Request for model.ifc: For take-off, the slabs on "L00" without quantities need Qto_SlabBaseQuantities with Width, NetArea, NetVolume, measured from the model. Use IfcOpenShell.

First a look at what the model holds.

```python
import ifcopenshell
import ifcopenshell.util.element
import ifcopenshell.util.unit

model = ifcopenshell.open("model.ifc")
print(model.schema)
for unit_type in ("LENGTHUNIT", "AREAUNIT", "VOLUMEUNIT"):
    print(unit_type, ifcopenshell.util.unit.calculate_unit_scale(model, unit_type))
storey = next(s for s in model.by_type("IfcBuildingStorey") if s.Name == "L00")
slabs = [e for e in ifcopenshell.util.element.get_decomposition(storey) if e.is_a("IfcSlab")]
for e in sorted(slabs, key=lambda e: e.id()):
    print(e.id(), e.is_a(), e.Name, list(ifcopenshell.util.element.get_psets(e, qtos_only=True)), sep=" | ")
```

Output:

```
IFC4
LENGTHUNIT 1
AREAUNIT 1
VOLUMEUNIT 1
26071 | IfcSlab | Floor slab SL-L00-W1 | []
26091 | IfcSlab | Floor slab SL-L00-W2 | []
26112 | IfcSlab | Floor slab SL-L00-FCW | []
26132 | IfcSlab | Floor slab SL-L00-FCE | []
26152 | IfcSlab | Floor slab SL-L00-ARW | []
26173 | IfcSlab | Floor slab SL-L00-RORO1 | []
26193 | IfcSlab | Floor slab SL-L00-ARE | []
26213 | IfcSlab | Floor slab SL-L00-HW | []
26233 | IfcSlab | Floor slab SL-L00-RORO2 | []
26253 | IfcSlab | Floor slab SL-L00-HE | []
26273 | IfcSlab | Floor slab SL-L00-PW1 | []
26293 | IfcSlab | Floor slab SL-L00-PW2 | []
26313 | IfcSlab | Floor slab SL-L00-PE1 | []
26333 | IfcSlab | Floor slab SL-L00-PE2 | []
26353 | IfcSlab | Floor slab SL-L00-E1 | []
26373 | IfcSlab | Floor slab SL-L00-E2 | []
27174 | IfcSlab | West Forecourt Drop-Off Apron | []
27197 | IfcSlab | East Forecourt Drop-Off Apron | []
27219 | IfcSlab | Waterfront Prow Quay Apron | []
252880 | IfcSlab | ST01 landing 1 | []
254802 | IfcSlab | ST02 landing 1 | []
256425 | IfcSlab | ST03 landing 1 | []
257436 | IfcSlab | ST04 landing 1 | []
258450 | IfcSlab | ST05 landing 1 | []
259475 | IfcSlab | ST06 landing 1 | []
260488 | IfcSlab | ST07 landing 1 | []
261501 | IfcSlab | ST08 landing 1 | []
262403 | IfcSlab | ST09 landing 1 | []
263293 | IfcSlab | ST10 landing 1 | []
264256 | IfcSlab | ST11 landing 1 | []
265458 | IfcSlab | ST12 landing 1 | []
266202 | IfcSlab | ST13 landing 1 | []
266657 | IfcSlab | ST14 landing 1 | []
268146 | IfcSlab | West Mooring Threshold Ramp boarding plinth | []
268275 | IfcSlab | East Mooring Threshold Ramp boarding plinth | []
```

```python
import ifcopenshell
import ifcopenshell.api.pset
import ifcopenshell.geom
import ifcopenshell.util.element
import ifcopenshell.util.shape
import ifcopenshell.util.unit

model = ifcopenshell.open("model.ifc")
unit_scale = ifcopenshell.util.unit.calculate_unit_scale(model)
area_scale = ifcopenshell.util.unit.calculate_unit_scale(model, "AREAUNIT")
volume_scale = ifcopenshell.util.unit.calculate_unit_scale(model, "VOLUMEUNIT")
settings = ifcopenshell.geom.settings()

storey = next(s for s in model.by_type("IfcBuildingStorey") if s.Name == "L00")
slabs = [e for e in ifcopenshell.util.element.get_decomposition(storey) if e.is_a("IfcSlab")]

for e in sorted(slabs, key=lambda e: e.id()):
    if ifcopenshell.util.element.get_psets(e, qtos_only=True, should_inherit=False):
        continue
    # Geometry comes back in metres, in the element's own axes.
    shape = ifcopenshell.geom.create_shape(settings, e)
    values = {
        "Width": ifcopenshell.util.shape.get_z(shape.geometry) / unit_scale,
        "NetArea": ifcopenshell.util.shape.get_footprint_area(shape.geometry) / area_scale,
        "NetVolume": ifcopenshell.util.shape.get_volume(shape.geometry) / volume_scale,
    }
    qto = ifcopenshell.api.pset.add_qto(model, product=e, name="Qto_SlabBaseQuantities")
    ifcopenshell.api.pset.edit_qto(model, qto=qto, properties=values)
    print(e.id(), {k: round(v, 3) for k, v in values.items()})

model.write("model_v2.ifc")
```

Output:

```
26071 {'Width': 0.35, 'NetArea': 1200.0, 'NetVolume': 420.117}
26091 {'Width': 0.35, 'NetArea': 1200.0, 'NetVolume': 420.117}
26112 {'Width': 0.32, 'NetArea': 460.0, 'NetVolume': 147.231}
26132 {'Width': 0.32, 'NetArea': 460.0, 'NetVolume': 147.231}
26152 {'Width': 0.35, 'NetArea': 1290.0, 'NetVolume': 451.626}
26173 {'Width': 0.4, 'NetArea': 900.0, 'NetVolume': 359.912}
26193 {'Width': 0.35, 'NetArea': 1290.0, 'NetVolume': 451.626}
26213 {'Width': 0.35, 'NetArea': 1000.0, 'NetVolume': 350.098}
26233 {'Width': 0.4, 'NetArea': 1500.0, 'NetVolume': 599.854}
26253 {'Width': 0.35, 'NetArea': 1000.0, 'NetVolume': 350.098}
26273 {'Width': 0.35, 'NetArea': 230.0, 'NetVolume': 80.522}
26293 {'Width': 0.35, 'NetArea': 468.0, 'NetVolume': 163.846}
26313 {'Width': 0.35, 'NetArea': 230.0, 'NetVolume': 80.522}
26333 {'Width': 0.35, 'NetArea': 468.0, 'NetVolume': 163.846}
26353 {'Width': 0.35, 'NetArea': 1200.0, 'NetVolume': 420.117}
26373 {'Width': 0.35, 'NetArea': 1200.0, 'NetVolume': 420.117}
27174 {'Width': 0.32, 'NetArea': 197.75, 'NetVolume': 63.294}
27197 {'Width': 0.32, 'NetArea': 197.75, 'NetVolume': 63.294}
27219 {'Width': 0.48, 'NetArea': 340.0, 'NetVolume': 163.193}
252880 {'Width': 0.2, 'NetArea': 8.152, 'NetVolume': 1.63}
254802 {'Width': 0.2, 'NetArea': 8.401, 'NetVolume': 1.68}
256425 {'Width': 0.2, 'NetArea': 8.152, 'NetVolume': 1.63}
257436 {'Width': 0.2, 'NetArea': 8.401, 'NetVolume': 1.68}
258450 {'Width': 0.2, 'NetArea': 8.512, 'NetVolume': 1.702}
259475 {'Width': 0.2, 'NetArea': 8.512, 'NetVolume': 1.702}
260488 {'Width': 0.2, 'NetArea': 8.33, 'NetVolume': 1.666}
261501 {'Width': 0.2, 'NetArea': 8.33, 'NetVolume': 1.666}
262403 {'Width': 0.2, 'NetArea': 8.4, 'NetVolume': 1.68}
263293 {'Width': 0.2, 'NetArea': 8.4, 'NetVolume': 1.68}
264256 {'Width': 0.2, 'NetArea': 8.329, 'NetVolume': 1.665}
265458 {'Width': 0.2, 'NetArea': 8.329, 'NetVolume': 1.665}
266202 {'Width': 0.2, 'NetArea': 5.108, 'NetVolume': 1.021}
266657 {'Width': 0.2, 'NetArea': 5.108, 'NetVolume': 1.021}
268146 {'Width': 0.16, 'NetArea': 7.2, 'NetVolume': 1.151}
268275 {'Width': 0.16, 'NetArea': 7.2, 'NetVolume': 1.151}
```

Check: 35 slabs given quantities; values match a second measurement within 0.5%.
